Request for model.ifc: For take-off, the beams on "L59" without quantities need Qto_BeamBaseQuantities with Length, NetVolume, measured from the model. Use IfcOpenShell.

First a look at what the model holds.

```python
import ifcopenshell
import ifcopenshell.util.element
import ifcopenshell.util.unit

model = ifcopenshell.open("model.ifc")
print(model.schema)
for unit_type in ("LENGTHUNIT", "AREAUNIT", "VOLUMEUNIT"):
    print(unit_type, ifcopenshell.util.unit.calculate_unit_scale(model, unit_type))
storey = next(s for s in model.by_type("IfcBuildingStorey") if s.Name == "L59")
beams = [e for e in ifcopenshell.util.element.get_decomposition(storey) if e.is_a("IfcBeam")]
for e in sorted(beams, key=lambda e: e.id()):
    print(e.id(), e.is_a(), e.Name, list(ifcopenshell.util.element.get_psets(e, qtos_only=True)), sep=" | ")
```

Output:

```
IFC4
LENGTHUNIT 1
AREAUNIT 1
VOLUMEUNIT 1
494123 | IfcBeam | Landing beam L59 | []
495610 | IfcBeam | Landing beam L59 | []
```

```python
import ifcopenshell
import ifcopenshell.api.pset
import ifcopenshell.geom
import ifcopenshell.util.element
import ifcopenshell.util.shape
import ifcopenshell.util.unit

model = ifcopenshell.open("model.ifc")
unit_scale = ifcopenshell.util.unit.calculate_unit_scale(model)
volume_scale = ifcopenshell.util.unit.calculate_unit_scale(model, "VOLUMEUNIT")
settings = ifcopenshell.geom.settings()

storey = next(s for s in model.by_type("IfcBuildingStorey") if s.Name == "L59")
beams = [e for e in ifcopenshell.util.element.get_decomposition(storey) if e.is_a("IfcBeam")]

for e in sorted(beams, key=lambda e: e.id()):
    if ifcopenshell.util.element.get_psets(e, qtos_only=True, should_inherit=False):
        continue
    # Geometry comes back in metres, in the element's own axes.
    shape = ifcopenshell.geom.create_shape(settings, e)
    values = {
        "Length": ifcopenshell.util.shape.get_max_xyz(shape.geometry) / unit_scale,
        "NetVolume": ifcopenshell.util.shape.get_volume(shape.geometry) / volume_scale,
    }
    qto = ifcopenshell.api.pset.add_qto(model, product=e, name="Qto_BeamBaseQuantities")
    ifcopenshell.api.pset.edit_qto(model, qto=qto, properties=values)
    print(e.id(), {k: round(v, 3) for k, v in values.items()})

model.write("model_updated.ifc")
```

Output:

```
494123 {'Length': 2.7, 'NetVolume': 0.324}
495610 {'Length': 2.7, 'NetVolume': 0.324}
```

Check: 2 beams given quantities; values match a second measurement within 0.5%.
